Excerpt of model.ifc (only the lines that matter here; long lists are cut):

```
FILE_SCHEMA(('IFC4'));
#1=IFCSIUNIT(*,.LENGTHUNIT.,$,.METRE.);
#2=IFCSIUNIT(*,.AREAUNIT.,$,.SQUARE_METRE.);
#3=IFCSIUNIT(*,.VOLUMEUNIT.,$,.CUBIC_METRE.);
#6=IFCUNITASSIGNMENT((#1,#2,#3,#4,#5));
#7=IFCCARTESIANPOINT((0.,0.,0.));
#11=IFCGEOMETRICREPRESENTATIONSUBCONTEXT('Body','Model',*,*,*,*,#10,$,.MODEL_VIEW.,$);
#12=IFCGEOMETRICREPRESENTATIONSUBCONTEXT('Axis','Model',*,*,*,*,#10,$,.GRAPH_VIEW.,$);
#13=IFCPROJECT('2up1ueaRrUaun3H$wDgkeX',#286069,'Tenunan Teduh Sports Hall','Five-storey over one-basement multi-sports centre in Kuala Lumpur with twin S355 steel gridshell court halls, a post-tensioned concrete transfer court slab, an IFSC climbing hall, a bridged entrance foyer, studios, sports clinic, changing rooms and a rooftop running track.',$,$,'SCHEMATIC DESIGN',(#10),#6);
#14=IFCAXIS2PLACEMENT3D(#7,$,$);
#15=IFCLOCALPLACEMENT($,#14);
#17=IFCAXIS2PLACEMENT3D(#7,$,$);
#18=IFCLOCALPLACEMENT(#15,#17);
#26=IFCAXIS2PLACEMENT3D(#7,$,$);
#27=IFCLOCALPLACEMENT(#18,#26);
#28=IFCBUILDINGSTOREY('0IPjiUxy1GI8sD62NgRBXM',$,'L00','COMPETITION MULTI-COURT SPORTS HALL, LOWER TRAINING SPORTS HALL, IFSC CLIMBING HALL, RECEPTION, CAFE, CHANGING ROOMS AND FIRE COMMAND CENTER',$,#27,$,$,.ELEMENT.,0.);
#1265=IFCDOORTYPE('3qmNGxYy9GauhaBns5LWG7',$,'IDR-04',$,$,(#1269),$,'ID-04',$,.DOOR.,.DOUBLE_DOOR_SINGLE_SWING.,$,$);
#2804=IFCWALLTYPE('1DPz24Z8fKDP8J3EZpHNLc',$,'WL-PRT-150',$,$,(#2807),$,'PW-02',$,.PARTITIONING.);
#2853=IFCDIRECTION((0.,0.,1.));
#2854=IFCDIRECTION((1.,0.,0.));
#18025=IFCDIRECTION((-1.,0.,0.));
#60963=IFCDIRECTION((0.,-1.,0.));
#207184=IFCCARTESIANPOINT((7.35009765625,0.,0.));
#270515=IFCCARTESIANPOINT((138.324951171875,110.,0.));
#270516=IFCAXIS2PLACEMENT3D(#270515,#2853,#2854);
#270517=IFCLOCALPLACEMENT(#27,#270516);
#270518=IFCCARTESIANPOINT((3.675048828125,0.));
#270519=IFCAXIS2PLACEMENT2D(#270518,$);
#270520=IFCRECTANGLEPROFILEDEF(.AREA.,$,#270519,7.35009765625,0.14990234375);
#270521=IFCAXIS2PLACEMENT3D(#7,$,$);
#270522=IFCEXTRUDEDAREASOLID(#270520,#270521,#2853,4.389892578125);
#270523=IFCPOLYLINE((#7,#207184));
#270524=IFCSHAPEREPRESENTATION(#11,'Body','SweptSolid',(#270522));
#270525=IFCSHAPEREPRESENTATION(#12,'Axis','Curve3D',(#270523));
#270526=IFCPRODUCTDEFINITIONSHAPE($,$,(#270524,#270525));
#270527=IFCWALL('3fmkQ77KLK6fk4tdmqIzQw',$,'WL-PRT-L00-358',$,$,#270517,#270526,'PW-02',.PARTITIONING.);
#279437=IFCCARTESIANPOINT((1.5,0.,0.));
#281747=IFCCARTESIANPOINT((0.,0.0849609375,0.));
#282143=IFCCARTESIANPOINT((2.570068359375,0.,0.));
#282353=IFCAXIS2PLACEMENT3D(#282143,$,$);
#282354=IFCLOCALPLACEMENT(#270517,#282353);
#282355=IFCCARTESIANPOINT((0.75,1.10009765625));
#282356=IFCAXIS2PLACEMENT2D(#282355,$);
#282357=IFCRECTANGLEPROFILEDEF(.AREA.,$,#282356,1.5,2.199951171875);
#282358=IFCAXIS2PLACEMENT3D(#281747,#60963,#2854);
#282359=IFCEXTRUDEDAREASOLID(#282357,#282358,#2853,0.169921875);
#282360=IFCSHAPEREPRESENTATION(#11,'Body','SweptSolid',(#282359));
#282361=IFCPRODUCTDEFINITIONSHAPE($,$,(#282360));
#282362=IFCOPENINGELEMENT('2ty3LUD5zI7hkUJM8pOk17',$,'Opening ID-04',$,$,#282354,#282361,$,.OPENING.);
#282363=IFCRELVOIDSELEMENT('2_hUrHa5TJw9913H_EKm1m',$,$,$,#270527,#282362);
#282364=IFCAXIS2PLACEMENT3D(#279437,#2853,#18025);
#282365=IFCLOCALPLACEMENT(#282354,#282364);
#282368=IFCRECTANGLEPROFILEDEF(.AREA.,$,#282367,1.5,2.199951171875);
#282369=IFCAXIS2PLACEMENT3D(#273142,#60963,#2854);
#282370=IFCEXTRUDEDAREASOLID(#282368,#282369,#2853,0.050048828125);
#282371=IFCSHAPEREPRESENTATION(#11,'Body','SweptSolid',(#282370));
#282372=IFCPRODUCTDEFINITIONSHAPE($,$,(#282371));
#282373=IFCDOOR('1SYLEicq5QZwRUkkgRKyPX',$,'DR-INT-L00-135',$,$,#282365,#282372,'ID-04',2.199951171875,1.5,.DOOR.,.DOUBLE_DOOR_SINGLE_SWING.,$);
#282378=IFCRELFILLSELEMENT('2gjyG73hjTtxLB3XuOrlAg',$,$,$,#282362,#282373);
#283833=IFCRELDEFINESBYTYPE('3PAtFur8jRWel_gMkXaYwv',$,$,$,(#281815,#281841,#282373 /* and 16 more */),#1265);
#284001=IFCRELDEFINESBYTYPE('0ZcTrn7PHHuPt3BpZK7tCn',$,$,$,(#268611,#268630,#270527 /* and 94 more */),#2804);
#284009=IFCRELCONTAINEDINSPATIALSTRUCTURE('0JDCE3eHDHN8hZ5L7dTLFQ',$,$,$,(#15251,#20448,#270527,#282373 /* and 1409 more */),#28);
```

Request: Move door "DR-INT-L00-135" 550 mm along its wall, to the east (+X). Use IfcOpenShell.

```python
import ifcopenshell
import ifcopenshell.api.geometry
import ifcopenshell.util.placement
import ifcopenshell.util.unit

model = ifcopenshell.open("model.ifc")
unit_scale = ifcopenshell.util.unit.calculate_unit_scale(model)

door = model.by_guid("1SYLEicq5QZwRUkkgRKyPX")
opening = door.FillsVoids[0].RelatingOpeningElement
wall = opening.VoidsElements[0].RelatingBuildingElement

wall_matrix = ifcopenshell.util.placement.get_local_placement(wall.ObjectPlacement)
shift = wall_matrix[:3, 0] * 0.55 / unit_scale
before = ifcopenshell.util.placement.get_local_placement(door.ObjectPlacement)[:3, 3].copy()

# The door is placed relative to its opening, so it follows when the opening moves.
matrix = ifcopenshell.util.placement.get_local_placement(opening.ObjectPlacement)
matrix[:3, 3] += shift
ifcopenshell.api.geometry.edit_object_placement(
    model, product=opening, matrix=matrix, is_si=False, should_transform_children=True
)

after = ifcopenshell.util.placement.get_local_placement(door.ObjectPlacement)[:3, 3]
print("door moved by", (after - before).round(3) + 0.0)

model.write("model_rev.ifc")
```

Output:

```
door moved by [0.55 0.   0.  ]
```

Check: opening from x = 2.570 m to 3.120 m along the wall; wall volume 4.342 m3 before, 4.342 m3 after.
